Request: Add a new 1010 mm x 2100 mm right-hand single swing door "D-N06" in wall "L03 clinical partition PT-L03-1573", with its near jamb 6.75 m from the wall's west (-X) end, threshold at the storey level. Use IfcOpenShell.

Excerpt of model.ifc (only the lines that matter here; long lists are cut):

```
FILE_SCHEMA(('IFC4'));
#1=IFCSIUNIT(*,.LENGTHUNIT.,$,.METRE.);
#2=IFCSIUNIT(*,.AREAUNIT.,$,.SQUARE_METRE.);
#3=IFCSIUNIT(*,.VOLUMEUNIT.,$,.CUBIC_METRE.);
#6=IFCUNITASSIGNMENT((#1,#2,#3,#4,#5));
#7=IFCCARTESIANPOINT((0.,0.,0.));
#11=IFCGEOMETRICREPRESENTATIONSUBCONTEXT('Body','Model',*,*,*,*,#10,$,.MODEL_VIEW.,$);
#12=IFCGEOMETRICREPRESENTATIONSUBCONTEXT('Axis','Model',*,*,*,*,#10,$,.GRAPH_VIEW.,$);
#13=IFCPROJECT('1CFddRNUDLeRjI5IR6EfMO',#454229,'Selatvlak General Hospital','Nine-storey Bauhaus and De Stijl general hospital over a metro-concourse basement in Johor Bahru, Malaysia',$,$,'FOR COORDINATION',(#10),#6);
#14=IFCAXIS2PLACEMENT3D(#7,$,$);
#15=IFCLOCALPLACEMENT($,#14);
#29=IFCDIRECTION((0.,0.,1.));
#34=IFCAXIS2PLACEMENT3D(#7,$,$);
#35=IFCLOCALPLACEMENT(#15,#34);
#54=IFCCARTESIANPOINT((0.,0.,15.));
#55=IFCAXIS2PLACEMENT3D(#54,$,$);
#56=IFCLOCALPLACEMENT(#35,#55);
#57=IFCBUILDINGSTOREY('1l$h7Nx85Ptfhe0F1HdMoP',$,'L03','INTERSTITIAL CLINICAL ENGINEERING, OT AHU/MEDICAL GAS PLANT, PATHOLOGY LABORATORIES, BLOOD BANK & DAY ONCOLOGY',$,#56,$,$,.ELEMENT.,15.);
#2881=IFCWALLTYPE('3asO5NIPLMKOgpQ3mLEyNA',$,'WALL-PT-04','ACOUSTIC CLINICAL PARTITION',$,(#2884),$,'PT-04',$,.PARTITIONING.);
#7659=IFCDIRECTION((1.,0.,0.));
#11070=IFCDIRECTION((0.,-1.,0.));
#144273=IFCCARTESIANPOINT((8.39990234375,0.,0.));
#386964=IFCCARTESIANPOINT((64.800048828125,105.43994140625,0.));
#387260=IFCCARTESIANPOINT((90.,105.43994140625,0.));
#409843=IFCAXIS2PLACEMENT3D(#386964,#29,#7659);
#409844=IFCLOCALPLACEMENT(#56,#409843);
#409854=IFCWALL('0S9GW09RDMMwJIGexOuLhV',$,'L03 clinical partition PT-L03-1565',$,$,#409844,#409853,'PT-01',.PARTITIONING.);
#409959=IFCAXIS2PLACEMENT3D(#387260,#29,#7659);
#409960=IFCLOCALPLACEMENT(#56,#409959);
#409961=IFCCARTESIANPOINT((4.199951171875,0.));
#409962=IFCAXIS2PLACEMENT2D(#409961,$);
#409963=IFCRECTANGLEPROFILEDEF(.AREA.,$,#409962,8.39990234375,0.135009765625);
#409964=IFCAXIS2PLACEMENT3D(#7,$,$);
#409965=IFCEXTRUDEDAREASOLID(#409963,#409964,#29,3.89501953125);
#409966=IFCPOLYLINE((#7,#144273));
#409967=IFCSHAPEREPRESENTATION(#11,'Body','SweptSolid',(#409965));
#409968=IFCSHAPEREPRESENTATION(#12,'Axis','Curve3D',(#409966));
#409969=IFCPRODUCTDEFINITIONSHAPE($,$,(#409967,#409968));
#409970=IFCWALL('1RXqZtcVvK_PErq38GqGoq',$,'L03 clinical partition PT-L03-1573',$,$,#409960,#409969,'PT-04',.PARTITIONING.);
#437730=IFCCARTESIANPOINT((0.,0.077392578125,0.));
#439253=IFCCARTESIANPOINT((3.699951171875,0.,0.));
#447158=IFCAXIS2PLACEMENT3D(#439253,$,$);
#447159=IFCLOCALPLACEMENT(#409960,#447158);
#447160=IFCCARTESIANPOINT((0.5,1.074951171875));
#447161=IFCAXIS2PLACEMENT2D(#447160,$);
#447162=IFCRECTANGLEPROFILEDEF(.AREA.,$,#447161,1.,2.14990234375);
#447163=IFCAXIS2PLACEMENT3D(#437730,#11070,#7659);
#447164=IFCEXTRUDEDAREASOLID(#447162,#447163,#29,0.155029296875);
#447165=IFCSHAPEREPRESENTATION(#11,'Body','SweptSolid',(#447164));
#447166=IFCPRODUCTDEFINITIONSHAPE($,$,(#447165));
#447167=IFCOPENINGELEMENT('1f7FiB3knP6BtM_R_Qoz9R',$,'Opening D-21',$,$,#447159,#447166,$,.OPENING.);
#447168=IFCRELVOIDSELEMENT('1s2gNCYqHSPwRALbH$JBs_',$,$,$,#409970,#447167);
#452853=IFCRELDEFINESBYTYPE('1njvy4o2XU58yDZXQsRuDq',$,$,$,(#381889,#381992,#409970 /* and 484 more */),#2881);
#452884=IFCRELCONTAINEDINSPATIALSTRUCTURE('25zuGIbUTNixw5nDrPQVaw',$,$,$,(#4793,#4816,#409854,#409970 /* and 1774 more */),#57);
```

```python
import numpy as np
import ifcopenshell
import ifcopenshell.api.feature
import ifcopenshell.api.geometry
import ifcopenshell.api.root
import ifcopenshell.api.spatial
import ifcopenshell.geom
import ifcopenshell.util.element
import ifcopenshell.util.placement
import ifcopenshell.util.representation
import ifcopenshell.util.shape
import ifcopenshell.util.unit

model = ifcopenshell.open("model.ifc")
unit_scale = ifcopenshell.util.unit.calculate_unit_scale(model)
settings = ifcopenshell.geom.settings()


def volume(element):
    """Net volume in cubic metres, openings subtracted."""
    shape = ifcopenshell.geom.create_shape(settings, element)
    return ifcopenshell.util.shape.get_volume(shape.geometry)


wall = model.by_guid("1RXqZtcVvK_PErq38GqGoq")
storey = ifcopenshell.util.element.get_container(wall, ifc_class="IfcBuildingStorey")
context = ifcopenshell.util.representation.get_context(model, "Model", "Body", "MODEL_VIEW")
before = volume(wall)

width, height, from_end, sill = 1.01, 2.1, 6.75, 0.0  # metres

# The wall runs along its own X axis, and the end named is its -X end.
wall_shape = ifcopenshell.geom.create_shape(settings, wall)
x, y, z = ifcopenshell.util.shape.get_vertices(wall_shape.geometry).T
start = x.min() + from_end
face, thickness = float(y.min()), float(y.max() - y.min())
wall_matrix = ifcopenshell.util.placement.get_local_placement(wall.ObjectPlacement)
level = ifcopenshell.util.placement.get_local_placement(storey.ObjectPlacement)[2, 3]


def in_wall(x, y):
    """Placement at x, y metres in the wall's axes, at sill height."""
    matrix = wall_matrix.copy()
    matrix[:, 3] = wall_matrix @ np.array([x / unit_scale, y / unit_scale, 0.0, 1.0])
    matrix[2, 3] = level + sill / unit_scale
    return matrix


# Opening: a box that overshoots both wall faces by 50 mm.
opening = ifcopenshell.api.root.create_entity(model, ifc_class="IfcOpeningElement", predefined_type="OPENING")
box = ifcopenshell.api.geometry.add_wall_representation(
    model, context=context, length=width, height=height, thickness=thickness + 0.1
)
ifcopenshell.api.geometry.assign_representation(model, product=opening, representation=box)
ifcopenshell.api.geometry.edit_object_placement(model, product=opening, matrix=in_wall(start, face - 0.05), is_si=False)
ifcopenshell.api.feature.add_feature(model, feature=opening, element=wall)

door = ifcopenshell.api.root.create_entity(model, ifc_class="IfcDoor", name="D-N06", predefined_type="DOOR")
door.OverallWidth, door.OverallHeight = width / unit_scale, height / unit_scale
door.OperationType = "SINGLE_SWING_RIGHT"
body = ifcopenshell.api.geometry.add_door_representation(
    model,
    context=context,
    overall_width=door.OverallWidth,
    overall_height=door.OverallHeight,
    operation_type="SINGLE_SWING_RIGHT",
    lining_properties={"LiningDepth": thickness / unit_scale, "ThresholdDepth": thickness / unit_scale},
)
ifcopenshell.api.geometry.assign_representation(model, product=door, representation=body)
ifcopenshell.api.spatial.assign_container(model, products=[door], relating_structure=storey)
ifcopenshell.api.feature.add_filling(model, opening=opening, element=door)

# The lining spans the wall, so the door starts at the wall face.
ifcopenshell.api.geometry.edit_object_placement(model, product=door, matrix=in_wall(start, face), is_si=False)

after = volume(wall)

print(f"wall volume {before:.3f} -> {after:.3f} m3")

model.write("model_edited.ifc")
```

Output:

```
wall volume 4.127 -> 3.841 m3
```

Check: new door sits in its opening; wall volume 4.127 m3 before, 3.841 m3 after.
